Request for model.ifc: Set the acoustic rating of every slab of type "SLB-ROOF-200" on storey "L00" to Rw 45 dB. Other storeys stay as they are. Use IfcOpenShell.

First a look at what the model holds.

```python
import ifcopenshell
import ifcopenshell.util.element

model = ifcopenshell.open("model.ifc")
print(model.schema)
storey = next(s for s in model.by_type("IfcBuildingStorey") if s.Name == "L00")
slabs = [e for e in ifcopenshell.util.element.get_decomposition(storey) if e.is_a("IfcSlab")]
seen = {}
for e in slabs:
    element_type = ifcopenshell.util.element.get_type(e)
    key = (element_type.Name if element_type != e and element_type else None, ifcopenshell.util.element.get_pset(e, "Pset_SlabCommon", "AcousticRating"))
    seen[key] = seen.get(key, 0) + 1
for (name, value), count in sorted(seen.items(), key=str):
    print(count, "x", name, "|", value)
```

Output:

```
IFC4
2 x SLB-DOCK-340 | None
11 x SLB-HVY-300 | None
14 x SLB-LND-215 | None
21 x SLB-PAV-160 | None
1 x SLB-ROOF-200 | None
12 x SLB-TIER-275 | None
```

```python
import ifcopenshell
import ifcopenshell.api.pset
import ifcopenshell.util.element

model = ifcopenshell.open("model.ifc")

storey = next(s for s in model.by_type("IfcBuildingStorey") if s.Name == "L00")
slabs = [e for e in ifcopenshell.util.element.get_decomposition(storey) if e.is_a("IfcSlab")]

count = 0
for e in slabs:
    element_type = ifcopenshell.util.element.get_type(e)
    if element_type in (None, e) or element_type.Name != "SLB-ROOF-200":
        continue
    # add_pset returns the element's existing set when there is one.
    pset = ifcopenshell.api.pset.add_pset(model, product=e, name="Pset_SlabCommon")
    ifcopenshell.api.pset.edit_pset(model, pset=pset, properties={"AcousticRating": "Rw 45 dB"})
    count += 1

print(count, "slabs updated")

model.write("model_v2.ifc")
```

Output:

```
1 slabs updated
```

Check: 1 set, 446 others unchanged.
